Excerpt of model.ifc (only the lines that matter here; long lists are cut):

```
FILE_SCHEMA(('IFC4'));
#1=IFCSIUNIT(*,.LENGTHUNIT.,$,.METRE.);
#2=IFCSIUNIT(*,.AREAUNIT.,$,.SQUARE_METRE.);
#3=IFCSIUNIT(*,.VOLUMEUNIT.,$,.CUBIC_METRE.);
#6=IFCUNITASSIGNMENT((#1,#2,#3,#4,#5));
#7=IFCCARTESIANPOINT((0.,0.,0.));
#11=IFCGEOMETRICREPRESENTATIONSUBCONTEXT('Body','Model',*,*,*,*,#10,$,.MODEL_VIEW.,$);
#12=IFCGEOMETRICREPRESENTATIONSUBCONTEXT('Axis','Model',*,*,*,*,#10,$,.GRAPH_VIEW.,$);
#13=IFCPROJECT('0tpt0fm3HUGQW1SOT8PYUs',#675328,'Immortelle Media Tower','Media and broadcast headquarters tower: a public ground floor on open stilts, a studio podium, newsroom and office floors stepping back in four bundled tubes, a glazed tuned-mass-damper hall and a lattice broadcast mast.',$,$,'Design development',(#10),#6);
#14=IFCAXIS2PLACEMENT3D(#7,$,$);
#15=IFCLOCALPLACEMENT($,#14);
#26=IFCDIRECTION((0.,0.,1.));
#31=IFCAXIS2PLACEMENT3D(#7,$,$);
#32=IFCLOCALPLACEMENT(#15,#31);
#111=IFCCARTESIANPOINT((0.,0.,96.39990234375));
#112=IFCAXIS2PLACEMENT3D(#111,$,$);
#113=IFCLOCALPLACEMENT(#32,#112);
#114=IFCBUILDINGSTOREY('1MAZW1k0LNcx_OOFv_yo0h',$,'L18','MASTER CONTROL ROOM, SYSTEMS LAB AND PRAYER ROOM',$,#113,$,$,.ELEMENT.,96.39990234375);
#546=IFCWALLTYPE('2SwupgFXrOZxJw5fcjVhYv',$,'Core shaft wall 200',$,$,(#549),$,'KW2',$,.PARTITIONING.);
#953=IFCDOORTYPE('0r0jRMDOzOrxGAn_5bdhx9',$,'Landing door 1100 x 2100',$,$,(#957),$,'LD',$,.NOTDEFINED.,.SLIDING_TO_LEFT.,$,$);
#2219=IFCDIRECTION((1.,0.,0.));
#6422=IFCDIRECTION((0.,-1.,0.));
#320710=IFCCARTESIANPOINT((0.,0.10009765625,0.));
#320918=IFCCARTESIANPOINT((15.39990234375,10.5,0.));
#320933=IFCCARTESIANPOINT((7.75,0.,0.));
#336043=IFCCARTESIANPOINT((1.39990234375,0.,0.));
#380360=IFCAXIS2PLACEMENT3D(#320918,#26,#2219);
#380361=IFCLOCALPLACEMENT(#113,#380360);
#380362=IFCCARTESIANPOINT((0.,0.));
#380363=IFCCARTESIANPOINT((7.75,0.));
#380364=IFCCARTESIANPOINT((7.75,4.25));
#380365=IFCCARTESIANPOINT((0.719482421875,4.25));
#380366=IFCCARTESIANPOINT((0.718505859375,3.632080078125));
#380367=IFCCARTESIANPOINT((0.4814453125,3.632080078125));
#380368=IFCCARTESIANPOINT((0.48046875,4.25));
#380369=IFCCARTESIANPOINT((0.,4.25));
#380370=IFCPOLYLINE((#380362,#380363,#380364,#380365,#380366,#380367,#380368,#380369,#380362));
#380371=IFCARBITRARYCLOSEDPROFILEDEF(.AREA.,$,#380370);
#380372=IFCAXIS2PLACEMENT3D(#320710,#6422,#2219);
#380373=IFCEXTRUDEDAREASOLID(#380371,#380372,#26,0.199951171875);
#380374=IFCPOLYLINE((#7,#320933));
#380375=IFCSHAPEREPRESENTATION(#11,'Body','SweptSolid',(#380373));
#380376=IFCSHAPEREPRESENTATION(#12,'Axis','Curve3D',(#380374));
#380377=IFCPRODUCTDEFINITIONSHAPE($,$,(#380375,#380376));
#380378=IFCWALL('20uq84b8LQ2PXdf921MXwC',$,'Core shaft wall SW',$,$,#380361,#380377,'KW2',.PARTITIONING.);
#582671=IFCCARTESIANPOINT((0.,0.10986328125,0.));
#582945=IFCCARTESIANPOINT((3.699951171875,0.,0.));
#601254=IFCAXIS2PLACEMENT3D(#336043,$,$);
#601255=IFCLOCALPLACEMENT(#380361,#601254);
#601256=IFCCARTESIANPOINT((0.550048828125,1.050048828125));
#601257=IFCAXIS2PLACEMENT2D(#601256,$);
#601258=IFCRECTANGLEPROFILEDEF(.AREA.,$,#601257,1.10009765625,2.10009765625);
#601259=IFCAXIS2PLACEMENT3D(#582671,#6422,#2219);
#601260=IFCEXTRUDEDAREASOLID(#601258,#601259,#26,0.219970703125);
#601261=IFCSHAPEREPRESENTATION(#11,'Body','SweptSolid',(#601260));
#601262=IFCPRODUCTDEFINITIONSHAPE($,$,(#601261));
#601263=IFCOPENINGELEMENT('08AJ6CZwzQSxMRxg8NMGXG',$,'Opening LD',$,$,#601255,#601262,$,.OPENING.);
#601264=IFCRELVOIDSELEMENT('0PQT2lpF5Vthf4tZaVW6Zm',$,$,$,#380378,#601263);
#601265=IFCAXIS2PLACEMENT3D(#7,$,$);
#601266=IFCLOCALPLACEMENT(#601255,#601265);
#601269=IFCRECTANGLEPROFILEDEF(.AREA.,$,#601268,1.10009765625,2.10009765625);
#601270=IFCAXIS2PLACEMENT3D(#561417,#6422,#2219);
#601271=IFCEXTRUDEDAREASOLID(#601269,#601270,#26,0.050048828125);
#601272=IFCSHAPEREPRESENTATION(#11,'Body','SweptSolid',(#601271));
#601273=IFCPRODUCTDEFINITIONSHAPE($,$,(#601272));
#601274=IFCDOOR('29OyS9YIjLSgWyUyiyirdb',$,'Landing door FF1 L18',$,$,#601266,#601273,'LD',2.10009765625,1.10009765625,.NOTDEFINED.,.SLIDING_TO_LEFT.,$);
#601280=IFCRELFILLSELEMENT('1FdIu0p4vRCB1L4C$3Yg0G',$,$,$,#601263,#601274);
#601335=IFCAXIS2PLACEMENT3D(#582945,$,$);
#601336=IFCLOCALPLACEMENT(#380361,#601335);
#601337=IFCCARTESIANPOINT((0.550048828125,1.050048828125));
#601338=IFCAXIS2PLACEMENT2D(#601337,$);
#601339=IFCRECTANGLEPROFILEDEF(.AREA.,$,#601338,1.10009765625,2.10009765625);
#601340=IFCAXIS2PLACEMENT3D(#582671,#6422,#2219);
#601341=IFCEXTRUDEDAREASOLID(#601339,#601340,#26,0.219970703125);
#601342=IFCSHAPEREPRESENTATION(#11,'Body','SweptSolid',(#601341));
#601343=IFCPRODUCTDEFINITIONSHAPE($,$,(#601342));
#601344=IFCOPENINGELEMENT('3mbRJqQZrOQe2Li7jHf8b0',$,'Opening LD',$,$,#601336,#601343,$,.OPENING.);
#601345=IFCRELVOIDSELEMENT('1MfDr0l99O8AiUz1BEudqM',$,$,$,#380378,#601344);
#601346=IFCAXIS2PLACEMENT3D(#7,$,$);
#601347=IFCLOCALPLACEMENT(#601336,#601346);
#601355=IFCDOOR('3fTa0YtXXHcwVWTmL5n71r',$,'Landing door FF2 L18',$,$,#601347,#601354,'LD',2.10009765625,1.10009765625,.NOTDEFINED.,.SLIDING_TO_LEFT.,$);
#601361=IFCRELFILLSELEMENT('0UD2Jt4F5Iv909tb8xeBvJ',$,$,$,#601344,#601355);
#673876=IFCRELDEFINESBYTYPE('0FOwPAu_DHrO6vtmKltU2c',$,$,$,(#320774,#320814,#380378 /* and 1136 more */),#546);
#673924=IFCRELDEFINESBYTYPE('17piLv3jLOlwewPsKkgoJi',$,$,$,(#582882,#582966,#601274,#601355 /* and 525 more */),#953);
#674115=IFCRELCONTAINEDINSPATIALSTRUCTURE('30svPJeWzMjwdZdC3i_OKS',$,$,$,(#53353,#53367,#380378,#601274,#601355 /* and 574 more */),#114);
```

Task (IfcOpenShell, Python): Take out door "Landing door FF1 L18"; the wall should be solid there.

```python
import ifcopenshell
import ifcopenshell.api.feature
import ifcopenshell.api.root
import ifcopenshell.geom
import ifcopenshell.util.shape

model = ifcopenshell.open("model.ifc")
settings = ifcopenshell.geom.settings()


def volume(element):
    """Net volume in cubic metres, openings subtracted."""
    shape = ifcopenshell.geom.create_shape(settings, element)
    return ifcopenshell.util.shape.get_volume(shape.geometry)


door = model.by_id(601274)
opening = door.FillsVoids[0].RelatingOpeningElement
wall = opening.VoidsElements[0].RelatingBuildingElement
before = volume(wall)

ifcopenshell.api.root.remove_product(model, product=door)
ifcopenshell.api.feature.remove_feature(model, feature=opening)

after = volume(wall)

print(f"wall volume {before:.3f} -> {after:.3f} m3")

model.write("model-out.ifc")
```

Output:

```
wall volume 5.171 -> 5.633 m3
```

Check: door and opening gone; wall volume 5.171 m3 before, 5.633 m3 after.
